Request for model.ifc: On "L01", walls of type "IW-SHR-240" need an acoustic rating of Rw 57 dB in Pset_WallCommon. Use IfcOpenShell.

First a look at what the model holds.

```python
import ifcopenshell
import ifcopenshell.util.element

model = ifcopenshell.open("model.ifc")
print(model.schema)
storey = next(s for s in model.by_type("IfcBuildingStorey") if s.Name == "L01")
walls = [e for e in ifcopenshell.util.element.get_decomposition(storey) if e.is_a("IfcWall")]
seen = {}
for e in walls:
    element_type = ifcopenshell.util.element.get_type(e)
    key = (element_type.Name if element_type != e and element_type else None, ifcopenshell.util.element.get_pset(e, "Pset_WallCommon", "AcousticRating"))
    seen[key] = seen.get(key, 0) + 1
for (name, value), count in sorted(seen.items(), key=str):
    print(count, "x", name, "|", value)
```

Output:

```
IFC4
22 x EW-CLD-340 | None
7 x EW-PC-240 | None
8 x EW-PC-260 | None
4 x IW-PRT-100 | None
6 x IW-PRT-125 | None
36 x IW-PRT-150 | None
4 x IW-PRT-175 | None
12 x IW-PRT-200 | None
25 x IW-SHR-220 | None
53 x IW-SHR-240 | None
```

```python
import ifcopenshell
import ifcopenshell.api.pset
import ifcopenshell.util.element

model = ifcopenshell.open("model.ifc")

storey = next(s for s in model.by_type("IfcBuildingStorey") if s.Name == "L01")
walls = [e for e in ifcopenshell.util.element.get_decomposition(storey) if e.is_a("IfcWall")]

count = 0
for e in walls:
    element_type = ifcopenshell.util.element.get_type(e)
    if element_type in (None, e) or element_type.Name != "IW-SHR-240":
        continue
    # add_pset returns the element's existing set when there is one.
    pset = ifcopenshell.api.pset.add_pset(model, product=e, name="Pset_WallCommon")
    ifcopenshell.api.pset.edit_pset(model, pset=pset, properties={"AcousticRating": "Rw 57 dB"})
    count += 1

print(count, "walls updated")

model.write("model_edited.ifc")
```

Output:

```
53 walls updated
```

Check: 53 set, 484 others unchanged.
